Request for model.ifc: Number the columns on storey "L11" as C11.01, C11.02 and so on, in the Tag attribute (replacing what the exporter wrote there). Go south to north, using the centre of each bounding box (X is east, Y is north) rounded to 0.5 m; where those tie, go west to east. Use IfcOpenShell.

First a look at what the model holds.

```python
import ifcopenshell
import ifcopenshell.util.element
import ifcopenshell.util.placement

model = ifcopenshell.open("model.ifc")
print(model.schema)
storey = next(s for s in model.by_type("IfcBuildingStorey") if s.Name == "L11")
columns = [e for e in ifcopenshell.util.element.get_decomposition(storey) if e.is_a("IfcColumn")]
for e in sorted(columns, key=lambda e: e.id()):
    origin = ifcopenshell.util.placement.get_local_placement(e.ObjectPlacement)[:3, 3]
    print(e.id(), e.Tag, e.Name, origin.round(2) + 0.0, sep=" | ")
```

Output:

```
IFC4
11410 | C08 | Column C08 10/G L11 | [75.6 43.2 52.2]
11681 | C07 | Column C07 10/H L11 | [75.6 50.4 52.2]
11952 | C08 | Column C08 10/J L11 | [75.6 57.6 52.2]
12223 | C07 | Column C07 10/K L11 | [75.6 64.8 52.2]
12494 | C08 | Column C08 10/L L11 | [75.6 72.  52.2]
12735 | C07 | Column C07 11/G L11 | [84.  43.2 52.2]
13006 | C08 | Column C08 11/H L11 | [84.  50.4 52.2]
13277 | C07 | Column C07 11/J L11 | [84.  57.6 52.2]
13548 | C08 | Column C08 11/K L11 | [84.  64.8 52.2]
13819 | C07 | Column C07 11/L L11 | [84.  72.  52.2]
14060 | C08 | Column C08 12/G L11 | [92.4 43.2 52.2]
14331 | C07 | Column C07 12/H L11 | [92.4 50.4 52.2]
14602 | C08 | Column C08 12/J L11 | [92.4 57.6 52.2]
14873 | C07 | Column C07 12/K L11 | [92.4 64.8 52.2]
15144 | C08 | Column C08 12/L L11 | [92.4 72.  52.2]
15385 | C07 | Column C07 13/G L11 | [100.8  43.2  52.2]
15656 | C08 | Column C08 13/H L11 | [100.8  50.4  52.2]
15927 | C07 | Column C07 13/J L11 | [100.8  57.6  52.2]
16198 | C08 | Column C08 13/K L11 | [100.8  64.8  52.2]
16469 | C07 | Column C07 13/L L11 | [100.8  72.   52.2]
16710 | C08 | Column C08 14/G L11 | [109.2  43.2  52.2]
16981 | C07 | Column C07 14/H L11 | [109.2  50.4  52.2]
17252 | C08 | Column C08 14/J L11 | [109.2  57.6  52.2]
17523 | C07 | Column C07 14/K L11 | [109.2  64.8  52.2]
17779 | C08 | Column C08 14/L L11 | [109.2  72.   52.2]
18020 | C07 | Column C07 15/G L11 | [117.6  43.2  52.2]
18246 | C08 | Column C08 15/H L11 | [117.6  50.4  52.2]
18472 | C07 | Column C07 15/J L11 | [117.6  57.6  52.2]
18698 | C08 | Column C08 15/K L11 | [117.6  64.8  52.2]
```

```python
import ifcopenshell
import ifcopenshell.geom
import ifcopenshell.util.element
import ifcopenshell.util.shape

model = ifcopenshell.open("model.ifc")
settings = ifcopenshell.geom.settings()
settings.set("use-world-coords", True)


def centre(element):
    shape = ifcopenshell.geom.create_shape(settings, element)
    return ifcopenshell.util.shape.get_bbox_centroid(shape.geometry)


storey = next(s for s in model.by_type("IfcBuildingStorey") if s.Name == "L11")
columns = [e for e in ifcopenshell.util.element.get_decomposition(storey) if e.is_a("IfcColumn")]

# Insertion points can sit at a corner or the storey origin, so sort by the geometry (in metres).
centres = {e: centre(e) for e in columns}
columns.sort(key=lambda e: (round(centres[e][1] / 0.5), centres[e][0]))

for i, e in enumerate(columns, start=1):
    number = f"C11.{i:02d}"
    e.Tag = number
    print(e.id(), number)

model.write("model_edited.ifc")
```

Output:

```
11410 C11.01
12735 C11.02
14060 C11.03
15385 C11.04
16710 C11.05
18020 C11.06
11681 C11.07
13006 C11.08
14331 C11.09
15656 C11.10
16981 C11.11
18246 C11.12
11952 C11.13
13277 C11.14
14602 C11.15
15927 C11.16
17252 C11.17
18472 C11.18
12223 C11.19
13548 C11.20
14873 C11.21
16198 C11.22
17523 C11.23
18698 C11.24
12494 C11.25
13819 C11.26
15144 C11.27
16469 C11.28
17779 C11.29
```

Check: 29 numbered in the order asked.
